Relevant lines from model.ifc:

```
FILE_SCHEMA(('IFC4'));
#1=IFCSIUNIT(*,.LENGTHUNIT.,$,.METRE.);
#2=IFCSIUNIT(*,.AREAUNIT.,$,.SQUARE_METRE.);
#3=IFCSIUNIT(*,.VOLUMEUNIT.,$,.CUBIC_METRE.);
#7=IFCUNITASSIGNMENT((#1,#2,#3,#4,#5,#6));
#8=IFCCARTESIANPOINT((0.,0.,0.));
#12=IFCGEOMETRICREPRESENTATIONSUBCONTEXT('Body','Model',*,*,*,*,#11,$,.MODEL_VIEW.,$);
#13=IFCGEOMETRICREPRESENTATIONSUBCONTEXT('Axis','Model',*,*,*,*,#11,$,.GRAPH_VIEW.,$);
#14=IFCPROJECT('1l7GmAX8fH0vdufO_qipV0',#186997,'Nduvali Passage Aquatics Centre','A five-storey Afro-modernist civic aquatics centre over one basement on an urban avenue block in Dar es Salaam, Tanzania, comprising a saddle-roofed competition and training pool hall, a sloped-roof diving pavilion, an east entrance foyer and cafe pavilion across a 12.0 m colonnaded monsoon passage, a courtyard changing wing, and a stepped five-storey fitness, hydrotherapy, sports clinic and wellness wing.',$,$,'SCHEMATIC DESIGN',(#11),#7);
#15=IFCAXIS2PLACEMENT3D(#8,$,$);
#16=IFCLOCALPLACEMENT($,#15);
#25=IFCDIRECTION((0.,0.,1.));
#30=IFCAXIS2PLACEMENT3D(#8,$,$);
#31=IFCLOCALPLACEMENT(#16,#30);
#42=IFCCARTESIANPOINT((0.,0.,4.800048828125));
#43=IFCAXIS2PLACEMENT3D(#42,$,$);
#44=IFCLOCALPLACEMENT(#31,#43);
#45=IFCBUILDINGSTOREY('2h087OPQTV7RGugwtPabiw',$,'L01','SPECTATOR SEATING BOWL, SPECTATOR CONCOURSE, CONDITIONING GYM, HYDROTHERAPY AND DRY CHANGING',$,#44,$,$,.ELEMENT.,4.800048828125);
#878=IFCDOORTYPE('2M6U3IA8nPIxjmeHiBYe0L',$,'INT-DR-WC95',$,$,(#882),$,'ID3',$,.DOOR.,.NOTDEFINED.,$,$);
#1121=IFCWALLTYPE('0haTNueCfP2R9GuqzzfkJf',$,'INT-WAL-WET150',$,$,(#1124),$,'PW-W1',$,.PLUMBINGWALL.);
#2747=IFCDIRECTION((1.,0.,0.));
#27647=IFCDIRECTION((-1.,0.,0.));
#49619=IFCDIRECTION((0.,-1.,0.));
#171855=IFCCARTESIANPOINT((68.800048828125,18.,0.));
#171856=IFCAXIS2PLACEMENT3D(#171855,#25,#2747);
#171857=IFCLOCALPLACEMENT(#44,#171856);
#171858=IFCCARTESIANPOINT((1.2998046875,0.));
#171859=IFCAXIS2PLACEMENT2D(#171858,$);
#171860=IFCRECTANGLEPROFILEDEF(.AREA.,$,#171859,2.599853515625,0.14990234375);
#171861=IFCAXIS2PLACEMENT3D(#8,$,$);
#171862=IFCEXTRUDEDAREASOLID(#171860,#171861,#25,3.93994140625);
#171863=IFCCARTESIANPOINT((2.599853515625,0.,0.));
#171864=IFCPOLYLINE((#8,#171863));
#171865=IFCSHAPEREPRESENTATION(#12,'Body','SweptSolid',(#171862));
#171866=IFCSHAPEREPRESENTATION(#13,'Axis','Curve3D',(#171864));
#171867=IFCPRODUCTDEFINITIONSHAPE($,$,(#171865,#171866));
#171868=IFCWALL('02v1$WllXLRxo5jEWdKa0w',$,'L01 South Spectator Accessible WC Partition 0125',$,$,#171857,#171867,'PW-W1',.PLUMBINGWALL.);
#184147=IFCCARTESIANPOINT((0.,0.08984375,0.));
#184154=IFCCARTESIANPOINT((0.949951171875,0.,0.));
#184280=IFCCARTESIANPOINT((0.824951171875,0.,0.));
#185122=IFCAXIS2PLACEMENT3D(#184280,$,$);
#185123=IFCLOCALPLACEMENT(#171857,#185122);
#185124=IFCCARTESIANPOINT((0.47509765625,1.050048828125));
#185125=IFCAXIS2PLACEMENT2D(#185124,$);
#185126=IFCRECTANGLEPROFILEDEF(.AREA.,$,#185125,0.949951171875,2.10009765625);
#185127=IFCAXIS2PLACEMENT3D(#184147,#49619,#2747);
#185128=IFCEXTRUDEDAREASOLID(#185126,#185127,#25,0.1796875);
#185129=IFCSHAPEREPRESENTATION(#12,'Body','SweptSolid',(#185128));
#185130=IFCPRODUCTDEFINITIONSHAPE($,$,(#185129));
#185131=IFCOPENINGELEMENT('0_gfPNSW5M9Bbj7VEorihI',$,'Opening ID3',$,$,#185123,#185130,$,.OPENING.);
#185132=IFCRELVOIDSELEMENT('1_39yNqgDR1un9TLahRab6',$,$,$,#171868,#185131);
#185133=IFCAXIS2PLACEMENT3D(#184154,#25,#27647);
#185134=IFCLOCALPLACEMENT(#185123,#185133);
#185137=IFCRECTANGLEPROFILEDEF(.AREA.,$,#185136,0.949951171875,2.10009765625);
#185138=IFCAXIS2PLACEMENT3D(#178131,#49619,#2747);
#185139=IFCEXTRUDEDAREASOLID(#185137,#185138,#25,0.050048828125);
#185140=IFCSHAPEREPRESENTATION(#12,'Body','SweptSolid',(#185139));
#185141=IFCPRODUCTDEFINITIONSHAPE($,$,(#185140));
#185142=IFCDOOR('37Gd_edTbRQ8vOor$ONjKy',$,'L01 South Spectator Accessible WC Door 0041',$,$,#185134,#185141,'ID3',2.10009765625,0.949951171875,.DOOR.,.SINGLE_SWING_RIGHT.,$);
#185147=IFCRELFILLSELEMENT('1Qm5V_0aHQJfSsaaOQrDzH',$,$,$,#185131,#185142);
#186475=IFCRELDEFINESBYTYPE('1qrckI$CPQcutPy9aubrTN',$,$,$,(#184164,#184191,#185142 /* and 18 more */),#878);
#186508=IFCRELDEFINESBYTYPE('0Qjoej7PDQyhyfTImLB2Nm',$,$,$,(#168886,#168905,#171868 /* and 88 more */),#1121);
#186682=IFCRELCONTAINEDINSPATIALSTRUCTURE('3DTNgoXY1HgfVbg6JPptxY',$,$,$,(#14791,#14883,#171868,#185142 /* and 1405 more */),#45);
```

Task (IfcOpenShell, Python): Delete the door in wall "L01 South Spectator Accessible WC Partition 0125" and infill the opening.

```python
import ifcopenshell
import ifcopenshell.api.feature
import ifcopenshell.api.root
import ifcopenshell.geom
import ifcopenshell.util.shape

model = ifcopenshell.open("model.ifc")
settings = ifcopenshell.geom.settings()


def volume(element):
    """Net volume in cubic metres, openings subtracted."""
    shape = ifcopenshell.geom.create_shape(settings, element)
    return ifcopenshell.util.shape.get_volume(shape.geometry)


door = model.by_guid("37Gd_edTbRQ8vOor$ONjKy")
opening = door.FillsVoids[0].RelatingOpeningElement
wall = opening.VoidsElements[0].RelatingBuildingElement
before = volume(wall)

ifcopenshell.api.root.remove_product(model, product=door)
ifcopenshell.api.feature.remove_feature(model, feature=opening)

after = volume(wall)

print(f"wall volume {before:.3f} -> {after:.3f} m3")

model.write("model_edited.ifc")
```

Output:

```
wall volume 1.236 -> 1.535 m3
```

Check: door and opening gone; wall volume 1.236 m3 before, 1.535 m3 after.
